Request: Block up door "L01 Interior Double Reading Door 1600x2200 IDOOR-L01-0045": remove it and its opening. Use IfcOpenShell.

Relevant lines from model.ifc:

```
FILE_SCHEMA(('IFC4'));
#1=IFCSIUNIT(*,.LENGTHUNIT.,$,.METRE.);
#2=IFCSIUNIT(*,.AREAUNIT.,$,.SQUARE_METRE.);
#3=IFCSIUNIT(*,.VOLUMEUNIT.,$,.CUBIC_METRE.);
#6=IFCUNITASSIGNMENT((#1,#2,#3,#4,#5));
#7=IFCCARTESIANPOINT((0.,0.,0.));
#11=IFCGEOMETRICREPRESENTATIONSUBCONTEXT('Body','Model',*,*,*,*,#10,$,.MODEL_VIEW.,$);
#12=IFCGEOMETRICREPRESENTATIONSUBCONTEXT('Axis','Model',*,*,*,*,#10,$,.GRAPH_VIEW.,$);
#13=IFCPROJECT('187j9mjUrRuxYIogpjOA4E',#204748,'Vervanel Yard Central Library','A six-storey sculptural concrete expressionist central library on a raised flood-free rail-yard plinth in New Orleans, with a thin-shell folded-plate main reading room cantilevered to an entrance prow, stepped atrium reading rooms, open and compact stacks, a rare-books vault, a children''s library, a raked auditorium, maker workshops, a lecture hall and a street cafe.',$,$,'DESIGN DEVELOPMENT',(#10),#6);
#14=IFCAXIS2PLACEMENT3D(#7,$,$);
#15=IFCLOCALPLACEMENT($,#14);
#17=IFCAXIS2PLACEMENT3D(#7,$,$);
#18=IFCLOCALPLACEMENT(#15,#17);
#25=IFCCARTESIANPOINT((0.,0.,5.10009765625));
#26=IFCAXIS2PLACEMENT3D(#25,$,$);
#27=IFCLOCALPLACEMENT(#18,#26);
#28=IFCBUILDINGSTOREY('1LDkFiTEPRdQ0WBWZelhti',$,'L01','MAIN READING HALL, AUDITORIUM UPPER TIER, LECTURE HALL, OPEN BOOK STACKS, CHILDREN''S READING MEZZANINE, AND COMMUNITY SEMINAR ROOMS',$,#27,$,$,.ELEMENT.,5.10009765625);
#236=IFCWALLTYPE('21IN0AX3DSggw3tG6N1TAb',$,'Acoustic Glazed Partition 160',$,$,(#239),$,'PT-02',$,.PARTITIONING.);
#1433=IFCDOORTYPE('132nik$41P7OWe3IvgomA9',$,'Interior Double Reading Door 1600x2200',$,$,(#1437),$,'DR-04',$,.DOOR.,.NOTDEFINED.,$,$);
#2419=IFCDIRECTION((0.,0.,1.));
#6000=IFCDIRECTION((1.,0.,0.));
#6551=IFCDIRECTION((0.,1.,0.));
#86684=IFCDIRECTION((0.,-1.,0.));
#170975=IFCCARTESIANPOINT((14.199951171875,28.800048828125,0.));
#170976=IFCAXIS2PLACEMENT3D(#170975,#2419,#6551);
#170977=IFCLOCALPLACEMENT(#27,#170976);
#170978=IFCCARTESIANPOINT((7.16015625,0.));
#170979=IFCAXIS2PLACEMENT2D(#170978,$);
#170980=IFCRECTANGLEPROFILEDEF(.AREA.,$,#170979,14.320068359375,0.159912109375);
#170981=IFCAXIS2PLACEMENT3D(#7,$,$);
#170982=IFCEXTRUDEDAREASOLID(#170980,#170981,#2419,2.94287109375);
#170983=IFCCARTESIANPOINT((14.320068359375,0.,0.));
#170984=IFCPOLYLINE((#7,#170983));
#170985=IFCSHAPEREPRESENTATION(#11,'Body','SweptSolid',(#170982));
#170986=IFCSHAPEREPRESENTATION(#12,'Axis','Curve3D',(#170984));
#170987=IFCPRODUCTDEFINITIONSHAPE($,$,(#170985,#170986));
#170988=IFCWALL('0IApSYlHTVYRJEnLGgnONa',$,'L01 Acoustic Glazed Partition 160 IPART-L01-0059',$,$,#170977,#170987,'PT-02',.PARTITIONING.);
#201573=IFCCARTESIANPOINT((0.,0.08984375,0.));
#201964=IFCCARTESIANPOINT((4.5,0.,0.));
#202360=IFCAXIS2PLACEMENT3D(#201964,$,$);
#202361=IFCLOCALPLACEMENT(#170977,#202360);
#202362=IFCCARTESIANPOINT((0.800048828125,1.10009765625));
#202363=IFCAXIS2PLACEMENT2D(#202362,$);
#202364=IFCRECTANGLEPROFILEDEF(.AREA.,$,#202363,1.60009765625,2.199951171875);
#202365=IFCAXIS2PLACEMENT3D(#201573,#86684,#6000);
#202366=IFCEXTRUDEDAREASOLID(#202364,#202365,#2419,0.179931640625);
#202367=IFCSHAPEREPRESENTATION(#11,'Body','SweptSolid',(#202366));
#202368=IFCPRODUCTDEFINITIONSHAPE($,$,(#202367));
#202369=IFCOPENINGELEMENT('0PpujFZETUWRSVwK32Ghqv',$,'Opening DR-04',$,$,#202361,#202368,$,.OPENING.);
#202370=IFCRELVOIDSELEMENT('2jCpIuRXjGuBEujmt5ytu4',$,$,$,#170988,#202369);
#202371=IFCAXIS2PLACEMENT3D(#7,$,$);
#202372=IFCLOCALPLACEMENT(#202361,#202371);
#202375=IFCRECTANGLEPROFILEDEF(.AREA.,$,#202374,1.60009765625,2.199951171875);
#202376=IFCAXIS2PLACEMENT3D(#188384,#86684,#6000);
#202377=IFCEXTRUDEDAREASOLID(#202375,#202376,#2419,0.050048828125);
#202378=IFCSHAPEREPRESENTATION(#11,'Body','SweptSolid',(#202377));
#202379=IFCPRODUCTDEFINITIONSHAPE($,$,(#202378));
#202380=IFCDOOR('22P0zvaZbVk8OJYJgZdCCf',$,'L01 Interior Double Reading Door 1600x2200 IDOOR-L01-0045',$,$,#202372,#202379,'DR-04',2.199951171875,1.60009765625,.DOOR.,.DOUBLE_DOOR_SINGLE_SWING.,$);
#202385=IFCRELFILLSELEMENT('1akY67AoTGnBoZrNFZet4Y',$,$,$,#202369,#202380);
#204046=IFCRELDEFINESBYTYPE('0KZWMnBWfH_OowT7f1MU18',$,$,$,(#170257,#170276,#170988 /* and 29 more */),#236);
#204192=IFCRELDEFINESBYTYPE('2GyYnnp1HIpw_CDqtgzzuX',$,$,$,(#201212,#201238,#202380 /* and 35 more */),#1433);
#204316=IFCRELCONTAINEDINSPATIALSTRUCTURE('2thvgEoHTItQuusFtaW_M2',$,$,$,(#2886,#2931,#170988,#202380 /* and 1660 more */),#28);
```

```python
import ifcopenshell
import ifcopenshell.api.feature
import ifcopenshell.api.root
import ifcopenshell.geom
import ifcopenshell.util.shape

model = ifcopenshell.open("model.ifc")
settings = ifcopenshell.geom.settings()


def volume(element):
    """Net volume in cubic metres, openings subtracted."""
    shape = ifcopenshell.geom.create_shape(settings, element)
    return ifcopenshell.util.shape.get_volume(shape.geometry)


door = model.by_guid("22P0zvaZbVk8OJYJgZdCCf")
opening = door.FillsVoids[0].RelatingOpeningElement
wall = opening.VoidsElements[0].RelatingBuildingElement
before = volume(wall)

ifcopenshell.api.root.remove_product(model, product=door)
ifcopenshell.api.feature.remove_feature(model, feature=opening)

after = volume(wall)

print(f"wall volume {before:.3f} -> {after:.3f} m3")

model.write("model_edited.ifc")
```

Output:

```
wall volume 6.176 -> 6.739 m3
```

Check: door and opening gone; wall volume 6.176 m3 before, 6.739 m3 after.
